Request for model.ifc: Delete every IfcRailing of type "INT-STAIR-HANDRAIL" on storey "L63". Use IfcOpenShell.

First a look at what the model holds.

```python
import ifcopenshell
import ifcopenshell.util.element

model = ifcopenshell.open("model.ifc")
print(model.schema)
storey = next(s for s in model.by_type("IfcBuildingStorey") if s.Name == "L63")
railings = [e for e in ifcopenshell.util.element.get_decomposition(storey) if e.is_a("IfcRailing")]
seen = {}
for e in railings:
    element_type = ifcopenshell.util.element.get_type(e)
    name = element_type.Name if element_type not in (None, e) else None
    seen[name] = seen.get(name, 0) + 1
for name, count in sorted(seen.items(), key=str):
    print(count, "x", name)
```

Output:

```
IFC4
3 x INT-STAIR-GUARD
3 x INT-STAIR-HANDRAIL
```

```python
import ifcopenshell
import ifcopenshell.api.root
import ifcopenshell.util.element

model = ifcopenshell.open("model.ifc")

storey = next(s for s in model.by_type("IfcBuildingStorey") if s.Name == "L63")
railings = [e for e in ifcopenshell.util.element.get_decomposition(storey) if e.is_a("IfcRailing")]
targets = [e for e in railings if (t := ifcopenshell.util.element.get_type(e)) not in (None, e) and t.Name == "INT-STAIR-HANDRAIL"]

for e in targets:
    ifcopenshell.api.root.remove_product(model, product=e)
print(len(targets), "removed")

model.write("model-out.ifc")
```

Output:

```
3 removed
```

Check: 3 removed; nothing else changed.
